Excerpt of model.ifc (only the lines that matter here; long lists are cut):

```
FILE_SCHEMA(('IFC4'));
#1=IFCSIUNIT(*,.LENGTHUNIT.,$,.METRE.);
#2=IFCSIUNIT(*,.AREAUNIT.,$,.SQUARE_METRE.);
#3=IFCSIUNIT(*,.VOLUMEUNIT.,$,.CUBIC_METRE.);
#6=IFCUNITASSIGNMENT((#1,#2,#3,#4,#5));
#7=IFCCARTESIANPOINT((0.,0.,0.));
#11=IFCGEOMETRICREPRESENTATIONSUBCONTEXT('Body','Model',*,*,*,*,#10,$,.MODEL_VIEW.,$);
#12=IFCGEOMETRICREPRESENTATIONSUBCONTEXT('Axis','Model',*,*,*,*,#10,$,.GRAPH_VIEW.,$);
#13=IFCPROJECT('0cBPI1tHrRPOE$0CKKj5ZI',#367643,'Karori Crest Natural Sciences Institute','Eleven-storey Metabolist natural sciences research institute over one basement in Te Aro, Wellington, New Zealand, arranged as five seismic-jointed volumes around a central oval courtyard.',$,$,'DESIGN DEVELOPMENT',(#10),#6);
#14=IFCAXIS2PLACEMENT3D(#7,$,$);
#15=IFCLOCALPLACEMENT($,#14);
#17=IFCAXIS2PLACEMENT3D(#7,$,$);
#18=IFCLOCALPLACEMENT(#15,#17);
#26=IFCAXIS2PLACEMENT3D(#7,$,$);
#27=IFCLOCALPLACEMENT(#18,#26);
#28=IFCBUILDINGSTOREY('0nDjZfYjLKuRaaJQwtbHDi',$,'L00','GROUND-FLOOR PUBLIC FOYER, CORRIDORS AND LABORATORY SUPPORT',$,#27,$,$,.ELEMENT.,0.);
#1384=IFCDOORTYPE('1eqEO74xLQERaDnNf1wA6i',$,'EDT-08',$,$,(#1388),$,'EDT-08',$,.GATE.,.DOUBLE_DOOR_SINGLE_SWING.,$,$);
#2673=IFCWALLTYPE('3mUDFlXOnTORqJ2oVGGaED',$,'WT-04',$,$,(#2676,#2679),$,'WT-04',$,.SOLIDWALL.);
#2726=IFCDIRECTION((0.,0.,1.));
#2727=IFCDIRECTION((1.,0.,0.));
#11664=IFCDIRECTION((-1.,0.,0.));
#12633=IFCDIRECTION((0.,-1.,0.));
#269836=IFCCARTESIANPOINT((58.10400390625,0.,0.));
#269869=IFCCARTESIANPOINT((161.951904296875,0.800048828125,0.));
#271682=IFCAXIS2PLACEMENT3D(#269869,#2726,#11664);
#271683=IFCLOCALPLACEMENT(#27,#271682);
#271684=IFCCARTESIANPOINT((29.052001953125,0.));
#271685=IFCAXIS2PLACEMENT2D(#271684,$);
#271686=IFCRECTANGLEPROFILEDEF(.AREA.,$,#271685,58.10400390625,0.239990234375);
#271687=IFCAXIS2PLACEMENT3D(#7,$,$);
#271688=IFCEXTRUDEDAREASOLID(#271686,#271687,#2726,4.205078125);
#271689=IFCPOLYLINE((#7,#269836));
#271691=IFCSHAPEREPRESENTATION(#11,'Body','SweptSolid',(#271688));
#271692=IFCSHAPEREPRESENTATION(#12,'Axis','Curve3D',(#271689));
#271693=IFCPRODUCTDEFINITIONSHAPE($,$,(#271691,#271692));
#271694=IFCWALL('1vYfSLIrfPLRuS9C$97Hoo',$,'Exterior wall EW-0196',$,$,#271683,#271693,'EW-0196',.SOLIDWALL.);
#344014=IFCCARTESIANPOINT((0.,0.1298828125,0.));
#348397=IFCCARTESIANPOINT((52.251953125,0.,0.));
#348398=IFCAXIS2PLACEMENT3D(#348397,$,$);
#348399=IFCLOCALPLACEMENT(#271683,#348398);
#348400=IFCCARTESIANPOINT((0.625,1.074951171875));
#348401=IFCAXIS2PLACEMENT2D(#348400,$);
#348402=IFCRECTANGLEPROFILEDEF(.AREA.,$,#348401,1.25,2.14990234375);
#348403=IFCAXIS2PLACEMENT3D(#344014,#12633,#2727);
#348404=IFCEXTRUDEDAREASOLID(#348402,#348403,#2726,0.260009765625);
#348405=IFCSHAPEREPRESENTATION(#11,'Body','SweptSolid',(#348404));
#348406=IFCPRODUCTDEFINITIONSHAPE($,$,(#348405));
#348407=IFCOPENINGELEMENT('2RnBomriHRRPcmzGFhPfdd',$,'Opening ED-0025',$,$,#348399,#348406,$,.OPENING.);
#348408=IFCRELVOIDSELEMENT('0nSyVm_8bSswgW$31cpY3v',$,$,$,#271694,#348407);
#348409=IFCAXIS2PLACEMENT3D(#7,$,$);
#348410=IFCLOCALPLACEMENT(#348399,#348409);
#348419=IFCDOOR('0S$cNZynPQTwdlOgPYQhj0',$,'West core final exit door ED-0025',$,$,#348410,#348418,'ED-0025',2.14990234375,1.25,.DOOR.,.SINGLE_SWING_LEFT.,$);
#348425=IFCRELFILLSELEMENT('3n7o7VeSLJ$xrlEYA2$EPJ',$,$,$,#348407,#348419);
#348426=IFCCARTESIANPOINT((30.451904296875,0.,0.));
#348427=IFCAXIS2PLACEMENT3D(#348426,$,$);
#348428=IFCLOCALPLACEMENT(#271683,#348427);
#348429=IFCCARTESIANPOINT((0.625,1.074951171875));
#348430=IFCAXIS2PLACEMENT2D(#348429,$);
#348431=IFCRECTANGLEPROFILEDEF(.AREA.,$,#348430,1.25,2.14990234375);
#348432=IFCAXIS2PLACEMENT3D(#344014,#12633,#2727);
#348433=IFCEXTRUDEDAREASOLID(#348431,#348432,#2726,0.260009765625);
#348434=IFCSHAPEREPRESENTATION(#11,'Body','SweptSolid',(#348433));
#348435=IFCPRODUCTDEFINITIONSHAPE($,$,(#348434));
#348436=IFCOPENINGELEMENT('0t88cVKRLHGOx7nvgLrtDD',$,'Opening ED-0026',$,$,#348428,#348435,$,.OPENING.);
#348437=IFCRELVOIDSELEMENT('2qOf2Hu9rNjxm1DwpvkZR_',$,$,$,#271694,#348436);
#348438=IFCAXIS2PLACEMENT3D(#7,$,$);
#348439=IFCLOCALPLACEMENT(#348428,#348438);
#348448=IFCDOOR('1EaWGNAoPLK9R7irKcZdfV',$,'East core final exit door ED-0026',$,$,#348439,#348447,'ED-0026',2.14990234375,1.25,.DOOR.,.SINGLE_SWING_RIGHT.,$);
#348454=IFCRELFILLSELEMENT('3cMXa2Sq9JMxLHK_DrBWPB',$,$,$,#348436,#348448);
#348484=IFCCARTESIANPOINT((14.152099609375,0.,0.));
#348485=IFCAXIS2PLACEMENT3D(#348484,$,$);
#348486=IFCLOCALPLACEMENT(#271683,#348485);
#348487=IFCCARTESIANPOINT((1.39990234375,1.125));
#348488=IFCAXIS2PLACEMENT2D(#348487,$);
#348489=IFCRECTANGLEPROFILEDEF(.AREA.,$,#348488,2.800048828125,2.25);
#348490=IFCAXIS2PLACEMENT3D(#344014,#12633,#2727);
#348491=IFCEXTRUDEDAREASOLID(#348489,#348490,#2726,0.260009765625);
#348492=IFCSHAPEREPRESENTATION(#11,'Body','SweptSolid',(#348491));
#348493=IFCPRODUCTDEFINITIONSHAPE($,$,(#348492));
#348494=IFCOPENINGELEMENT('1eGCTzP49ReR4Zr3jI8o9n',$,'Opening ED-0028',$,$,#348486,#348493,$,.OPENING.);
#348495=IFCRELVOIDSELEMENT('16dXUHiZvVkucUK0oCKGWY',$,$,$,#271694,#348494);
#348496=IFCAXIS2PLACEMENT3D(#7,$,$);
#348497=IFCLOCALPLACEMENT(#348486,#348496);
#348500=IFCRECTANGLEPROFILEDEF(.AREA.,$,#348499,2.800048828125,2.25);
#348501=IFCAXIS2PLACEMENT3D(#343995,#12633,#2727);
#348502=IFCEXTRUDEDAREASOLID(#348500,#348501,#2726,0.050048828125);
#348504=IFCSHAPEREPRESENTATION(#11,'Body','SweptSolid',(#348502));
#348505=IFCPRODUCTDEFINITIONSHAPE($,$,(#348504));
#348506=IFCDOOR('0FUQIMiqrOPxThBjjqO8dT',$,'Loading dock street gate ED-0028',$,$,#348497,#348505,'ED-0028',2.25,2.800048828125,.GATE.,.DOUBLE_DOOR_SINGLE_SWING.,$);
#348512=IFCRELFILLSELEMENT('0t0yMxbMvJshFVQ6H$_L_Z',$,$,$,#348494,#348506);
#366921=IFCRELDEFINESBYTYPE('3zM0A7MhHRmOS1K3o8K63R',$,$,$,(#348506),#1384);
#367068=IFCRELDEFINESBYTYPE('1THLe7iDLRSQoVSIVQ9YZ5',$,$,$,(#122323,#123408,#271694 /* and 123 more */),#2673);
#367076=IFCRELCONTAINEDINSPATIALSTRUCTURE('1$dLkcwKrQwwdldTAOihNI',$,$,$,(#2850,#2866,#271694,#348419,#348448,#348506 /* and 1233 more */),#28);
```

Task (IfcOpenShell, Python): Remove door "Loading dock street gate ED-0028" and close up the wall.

```python
import ifcopenshell
import ifcopenshell.api.feature
import ifcopenshell.api.root
import ifcopenshell.geom
import ifcopenshell.util.shape

model = ifcopenshell.open("model.ifc")
settings = ifcopenshell.geom.settings()


def volume(element):
    """Net volume in cubic metres, openings subtracted."""
    shape = ifcopenshell.geom.create_shape(settings, element)
    return ifcopenshell.util.shape.get_volume(shape.geometry)


door = model.by_guid("0FUQIMiqrOPxThBjjqO8dT")
opening = door.FillsVoids[0].RelatingOpeningElement
wall = opening.VoidsElements[0].RelatingBuildingElement
before = volume(wall)

ifcopenshell.api.root.remove_product(model, product=door)
ifcopenshell.api.feature.remove_feature(model, feature=opening)

after = volume(wall)

print(f"wall volume {before:.3f} -> {after:.3f} m3")

model.write("model_edited.ifc")
```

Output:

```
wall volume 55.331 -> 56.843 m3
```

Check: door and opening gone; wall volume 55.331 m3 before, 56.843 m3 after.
